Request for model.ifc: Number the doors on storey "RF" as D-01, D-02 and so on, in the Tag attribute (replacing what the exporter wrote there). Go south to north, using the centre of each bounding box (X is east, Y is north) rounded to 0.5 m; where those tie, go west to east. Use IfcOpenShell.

First a look at what the model holds.

```python
import ifcopenshell
import ifcopenshell.util.element
import ifcopenshell.util.placement

model = ifcopenshell.open("model.ifc")
print(model.schema)
storey = next(s for s in model.by_type("IfcBuildingStorey") if s.Name == "RF")
doors = [e for e in ifcopenshell.util.element.get_decomposition(storey) if e.is_a("IfcDoor")]
for e in sorted(doors, key=lambda e: e.id()):
    origin = ifcopenshell.util.placement.get_local_placement(e.ObjectPlacement)[:3, 3]
    print(e.id(), e.Tag, e.Name, origin.round(2) + 0.0, sep=" | ")
```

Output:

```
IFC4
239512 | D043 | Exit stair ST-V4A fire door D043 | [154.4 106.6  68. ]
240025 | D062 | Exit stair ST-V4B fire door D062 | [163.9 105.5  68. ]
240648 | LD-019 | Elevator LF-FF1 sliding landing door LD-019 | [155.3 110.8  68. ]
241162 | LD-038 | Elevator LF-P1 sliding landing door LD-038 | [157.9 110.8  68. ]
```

```python
import ifcopenshell
import ifcopenshell.geom
import ifcopenshell.util.element
import ifcopenshell.util.shape

model = ifcopenshell.open("model.ifc")
settings = ifcopenshell.geom.settings()
settings.set("use-world-coords", True)


def centre(element):
    shape = ifcopenshell.geom.create_shape(settings, element)
    return ifcopenshell.util.shape.get_bbox_centroid(shape.geometry)


storey = next(s for s in model.by_type("IfcBuildingStorey") if s.Name == "RF")
doors = [e for e in ifcopenshell.util.element.get_decomposition(storey) if e.is_a("IfcDoor")]

# Insertion points can sit at a corner or the storey origin, so sort by the geometry (in metres).
centres = {e: centre(e) for e in doors}
doors.sort(key=lambda e: (round(centres[e][1] / 0.5), centres[e][0]))

for i, e in enumerate(doors, start=1):
    number = f"D-{i:02d}"
    e.Tag = number
    print(e.id(), number)

model.write("model_edited.ifc")
```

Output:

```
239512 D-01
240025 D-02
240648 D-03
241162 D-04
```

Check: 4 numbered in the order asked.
